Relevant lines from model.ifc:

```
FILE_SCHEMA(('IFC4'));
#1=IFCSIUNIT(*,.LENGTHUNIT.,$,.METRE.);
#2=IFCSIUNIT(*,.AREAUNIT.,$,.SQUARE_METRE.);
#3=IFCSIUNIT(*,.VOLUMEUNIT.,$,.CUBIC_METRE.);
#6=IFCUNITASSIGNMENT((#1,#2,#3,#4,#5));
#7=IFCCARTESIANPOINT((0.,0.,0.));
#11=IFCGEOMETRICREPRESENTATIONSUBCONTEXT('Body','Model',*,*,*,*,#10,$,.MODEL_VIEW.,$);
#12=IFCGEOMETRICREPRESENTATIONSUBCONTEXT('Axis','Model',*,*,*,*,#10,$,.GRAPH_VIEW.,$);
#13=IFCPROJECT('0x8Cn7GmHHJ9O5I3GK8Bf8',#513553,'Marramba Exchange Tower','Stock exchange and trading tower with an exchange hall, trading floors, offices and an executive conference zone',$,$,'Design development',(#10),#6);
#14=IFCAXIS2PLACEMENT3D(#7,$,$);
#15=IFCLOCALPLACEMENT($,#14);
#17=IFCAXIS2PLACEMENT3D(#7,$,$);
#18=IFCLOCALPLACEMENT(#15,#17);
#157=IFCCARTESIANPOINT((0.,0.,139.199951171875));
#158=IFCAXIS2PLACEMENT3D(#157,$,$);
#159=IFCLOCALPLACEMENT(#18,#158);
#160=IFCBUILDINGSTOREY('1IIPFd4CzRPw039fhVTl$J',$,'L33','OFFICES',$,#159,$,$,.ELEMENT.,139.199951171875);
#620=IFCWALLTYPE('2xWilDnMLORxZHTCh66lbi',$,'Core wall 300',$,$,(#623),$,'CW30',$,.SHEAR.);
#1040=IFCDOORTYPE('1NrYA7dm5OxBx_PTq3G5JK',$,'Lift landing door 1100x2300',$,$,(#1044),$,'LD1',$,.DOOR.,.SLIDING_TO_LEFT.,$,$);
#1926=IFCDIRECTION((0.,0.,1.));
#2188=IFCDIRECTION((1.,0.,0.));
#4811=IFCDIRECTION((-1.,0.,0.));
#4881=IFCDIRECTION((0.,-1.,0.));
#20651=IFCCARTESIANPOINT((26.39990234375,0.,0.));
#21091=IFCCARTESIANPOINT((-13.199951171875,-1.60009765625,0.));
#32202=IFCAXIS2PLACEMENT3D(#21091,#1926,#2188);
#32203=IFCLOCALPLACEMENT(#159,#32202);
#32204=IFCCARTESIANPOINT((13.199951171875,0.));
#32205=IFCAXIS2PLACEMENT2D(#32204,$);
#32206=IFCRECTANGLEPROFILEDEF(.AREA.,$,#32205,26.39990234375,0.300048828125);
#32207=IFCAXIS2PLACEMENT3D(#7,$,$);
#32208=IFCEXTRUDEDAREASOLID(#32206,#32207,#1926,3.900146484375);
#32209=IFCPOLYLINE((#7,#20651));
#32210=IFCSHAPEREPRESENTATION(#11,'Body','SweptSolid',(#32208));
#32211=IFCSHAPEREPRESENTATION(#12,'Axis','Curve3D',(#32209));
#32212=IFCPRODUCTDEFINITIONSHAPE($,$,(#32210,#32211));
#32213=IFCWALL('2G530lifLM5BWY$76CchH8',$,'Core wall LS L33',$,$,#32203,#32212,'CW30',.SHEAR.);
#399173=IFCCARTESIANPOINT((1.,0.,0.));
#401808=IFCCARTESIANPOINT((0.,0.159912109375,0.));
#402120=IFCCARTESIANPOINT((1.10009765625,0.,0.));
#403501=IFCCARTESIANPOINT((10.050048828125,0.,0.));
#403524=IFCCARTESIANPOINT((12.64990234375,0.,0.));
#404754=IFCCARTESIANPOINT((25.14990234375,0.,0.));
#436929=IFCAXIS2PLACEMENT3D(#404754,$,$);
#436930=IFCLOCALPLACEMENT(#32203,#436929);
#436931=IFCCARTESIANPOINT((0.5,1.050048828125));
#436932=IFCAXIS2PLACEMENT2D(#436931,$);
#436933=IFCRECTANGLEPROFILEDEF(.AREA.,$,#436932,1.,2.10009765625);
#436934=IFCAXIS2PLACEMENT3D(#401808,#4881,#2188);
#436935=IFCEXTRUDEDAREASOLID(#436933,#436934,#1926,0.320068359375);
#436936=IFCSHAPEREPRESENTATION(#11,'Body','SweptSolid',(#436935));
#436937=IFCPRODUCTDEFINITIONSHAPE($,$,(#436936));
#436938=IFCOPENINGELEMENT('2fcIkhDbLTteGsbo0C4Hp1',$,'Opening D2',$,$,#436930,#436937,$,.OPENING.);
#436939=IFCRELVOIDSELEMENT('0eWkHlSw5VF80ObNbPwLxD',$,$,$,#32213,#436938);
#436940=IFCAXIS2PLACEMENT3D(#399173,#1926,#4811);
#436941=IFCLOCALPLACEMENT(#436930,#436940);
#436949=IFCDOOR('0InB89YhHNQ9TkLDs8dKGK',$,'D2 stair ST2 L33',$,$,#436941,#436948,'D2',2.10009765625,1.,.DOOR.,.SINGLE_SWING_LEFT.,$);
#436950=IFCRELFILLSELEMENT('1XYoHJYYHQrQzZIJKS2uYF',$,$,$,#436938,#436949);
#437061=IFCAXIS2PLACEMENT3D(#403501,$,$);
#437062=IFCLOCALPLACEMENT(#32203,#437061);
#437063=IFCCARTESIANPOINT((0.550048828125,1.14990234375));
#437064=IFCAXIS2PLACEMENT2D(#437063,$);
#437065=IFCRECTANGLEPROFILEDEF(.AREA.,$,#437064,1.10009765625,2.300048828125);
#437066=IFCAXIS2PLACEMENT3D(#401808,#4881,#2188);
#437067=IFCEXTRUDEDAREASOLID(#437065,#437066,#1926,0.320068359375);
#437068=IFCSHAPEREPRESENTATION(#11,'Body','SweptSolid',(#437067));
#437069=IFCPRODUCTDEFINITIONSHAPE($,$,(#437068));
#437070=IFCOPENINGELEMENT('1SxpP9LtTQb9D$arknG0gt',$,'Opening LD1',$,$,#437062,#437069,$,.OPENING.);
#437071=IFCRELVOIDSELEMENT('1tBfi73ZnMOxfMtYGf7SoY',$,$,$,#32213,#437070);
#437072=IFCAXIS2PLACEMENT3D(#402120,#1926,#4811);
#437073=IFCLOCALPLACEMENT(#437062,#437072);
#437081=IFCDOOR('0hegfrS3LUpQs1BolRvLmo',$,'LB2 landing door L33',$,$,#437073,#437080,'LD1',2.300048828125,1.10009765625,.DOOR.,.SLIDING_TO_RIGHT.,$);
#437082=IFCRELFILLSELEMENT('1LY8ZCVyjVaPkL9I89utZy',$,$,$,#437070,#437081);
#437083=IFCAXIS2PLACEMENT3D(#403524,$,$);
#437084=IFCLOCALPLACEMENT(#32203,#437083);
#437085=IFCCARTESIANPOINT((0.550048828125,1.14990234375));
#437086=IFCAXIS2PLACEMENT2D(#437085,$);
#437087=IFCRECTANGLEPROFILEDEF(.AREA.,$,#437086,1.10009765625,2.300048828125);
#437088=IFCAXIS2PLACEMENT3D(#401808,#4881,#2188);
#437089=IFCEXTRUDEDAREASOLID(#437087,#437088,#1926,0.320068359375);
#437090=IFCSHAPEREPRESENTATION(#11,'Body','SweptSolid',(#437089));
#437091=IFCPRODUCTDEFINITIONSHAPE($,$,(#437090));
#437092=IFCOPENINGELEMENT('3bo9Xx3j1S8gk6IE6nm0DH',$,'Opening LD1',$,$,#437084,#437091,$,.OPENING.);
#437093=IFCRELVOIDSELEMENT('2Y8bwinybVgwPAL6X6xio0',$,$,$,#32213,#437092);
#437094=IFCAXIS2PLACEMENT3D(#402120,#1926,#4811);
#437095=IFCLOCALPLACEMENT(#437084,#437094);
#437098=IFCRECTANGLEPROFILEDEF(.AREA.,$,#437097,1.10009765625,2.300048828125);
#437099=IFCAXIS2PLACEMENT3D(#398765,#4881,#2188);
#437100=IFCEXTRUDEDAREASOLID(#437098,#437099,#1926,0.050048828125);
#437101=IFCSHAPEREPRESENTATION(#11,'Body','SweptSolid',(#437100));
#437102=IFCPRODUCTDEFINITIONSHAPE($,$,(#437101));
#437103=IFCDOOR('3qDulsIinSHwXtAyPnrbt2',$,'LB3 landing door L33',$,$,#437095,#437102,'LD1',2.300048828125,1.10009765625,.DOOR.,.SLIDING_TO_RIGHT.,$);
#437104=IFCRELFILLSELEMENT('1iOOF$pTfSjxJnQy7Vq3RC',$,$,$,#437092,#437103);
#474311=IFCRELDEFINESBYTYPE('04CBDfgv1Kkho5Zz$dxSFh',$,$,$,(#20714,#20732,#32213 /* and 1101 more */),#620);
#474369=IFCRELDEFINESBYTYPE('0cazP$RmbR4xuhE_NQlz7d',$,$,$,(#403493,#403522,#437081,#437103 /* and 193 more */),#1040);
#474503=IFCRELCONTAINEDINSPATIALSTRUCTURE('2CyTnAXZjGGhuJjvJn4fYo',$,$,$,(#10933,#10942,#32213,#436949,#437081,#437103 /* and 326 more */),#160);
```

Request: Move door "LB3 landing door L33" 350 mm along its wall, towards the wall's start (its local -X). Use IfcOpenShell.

```python
import ifcopenshell
import ifcopenshell.api.geometry
import ifcopenshell.util.placement
import ifcopenshell.util.unit

model = ifcopenshell.open("model.ifc")
unit_scale = ifcopenshell.util.unit.calculate_unit_scale(model)

door = model.by_guid("3qDulsIinSHwXtAyPnrbt2")
opening = door.FillsVoids[0].RelatingOpeningElement
wall = opening.VoidsElements[0].RelatingBuildingElement

wall_matrix = ifcopenshell.util.placement.get_local_placement(wall.ObjectPlacement)
shift = wall_matrix[:3, 0] * -0.35 / unit_scale
before = ifcopenshell.util.placement.get_local_placement(door.ObjectPlacement)[:3, 3].copy()

# The door is placed relative to its opening, so it follows when the opening moves.
matrix = ifcopenshell.util.placement.get_local_placement(opening.ObjectPlacement)
matrix[:3, 3] += shift
ifcopenshell.api.geometry.edit_object_placement(
    model, product=opening, matrix=matrix, is_si=False, should_transform_children=True
)

after = ifcopenshell.util.placement.get_local_placement(door.ObjectPlacement)[:3, 3]
print("door moved by", (after - before).round(3) + 0.0)

model.write("model_edited.ifc")
```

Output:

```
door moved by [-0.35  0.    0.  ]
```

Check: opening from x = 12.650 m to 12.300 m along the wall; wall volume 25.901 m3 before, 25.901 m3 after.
